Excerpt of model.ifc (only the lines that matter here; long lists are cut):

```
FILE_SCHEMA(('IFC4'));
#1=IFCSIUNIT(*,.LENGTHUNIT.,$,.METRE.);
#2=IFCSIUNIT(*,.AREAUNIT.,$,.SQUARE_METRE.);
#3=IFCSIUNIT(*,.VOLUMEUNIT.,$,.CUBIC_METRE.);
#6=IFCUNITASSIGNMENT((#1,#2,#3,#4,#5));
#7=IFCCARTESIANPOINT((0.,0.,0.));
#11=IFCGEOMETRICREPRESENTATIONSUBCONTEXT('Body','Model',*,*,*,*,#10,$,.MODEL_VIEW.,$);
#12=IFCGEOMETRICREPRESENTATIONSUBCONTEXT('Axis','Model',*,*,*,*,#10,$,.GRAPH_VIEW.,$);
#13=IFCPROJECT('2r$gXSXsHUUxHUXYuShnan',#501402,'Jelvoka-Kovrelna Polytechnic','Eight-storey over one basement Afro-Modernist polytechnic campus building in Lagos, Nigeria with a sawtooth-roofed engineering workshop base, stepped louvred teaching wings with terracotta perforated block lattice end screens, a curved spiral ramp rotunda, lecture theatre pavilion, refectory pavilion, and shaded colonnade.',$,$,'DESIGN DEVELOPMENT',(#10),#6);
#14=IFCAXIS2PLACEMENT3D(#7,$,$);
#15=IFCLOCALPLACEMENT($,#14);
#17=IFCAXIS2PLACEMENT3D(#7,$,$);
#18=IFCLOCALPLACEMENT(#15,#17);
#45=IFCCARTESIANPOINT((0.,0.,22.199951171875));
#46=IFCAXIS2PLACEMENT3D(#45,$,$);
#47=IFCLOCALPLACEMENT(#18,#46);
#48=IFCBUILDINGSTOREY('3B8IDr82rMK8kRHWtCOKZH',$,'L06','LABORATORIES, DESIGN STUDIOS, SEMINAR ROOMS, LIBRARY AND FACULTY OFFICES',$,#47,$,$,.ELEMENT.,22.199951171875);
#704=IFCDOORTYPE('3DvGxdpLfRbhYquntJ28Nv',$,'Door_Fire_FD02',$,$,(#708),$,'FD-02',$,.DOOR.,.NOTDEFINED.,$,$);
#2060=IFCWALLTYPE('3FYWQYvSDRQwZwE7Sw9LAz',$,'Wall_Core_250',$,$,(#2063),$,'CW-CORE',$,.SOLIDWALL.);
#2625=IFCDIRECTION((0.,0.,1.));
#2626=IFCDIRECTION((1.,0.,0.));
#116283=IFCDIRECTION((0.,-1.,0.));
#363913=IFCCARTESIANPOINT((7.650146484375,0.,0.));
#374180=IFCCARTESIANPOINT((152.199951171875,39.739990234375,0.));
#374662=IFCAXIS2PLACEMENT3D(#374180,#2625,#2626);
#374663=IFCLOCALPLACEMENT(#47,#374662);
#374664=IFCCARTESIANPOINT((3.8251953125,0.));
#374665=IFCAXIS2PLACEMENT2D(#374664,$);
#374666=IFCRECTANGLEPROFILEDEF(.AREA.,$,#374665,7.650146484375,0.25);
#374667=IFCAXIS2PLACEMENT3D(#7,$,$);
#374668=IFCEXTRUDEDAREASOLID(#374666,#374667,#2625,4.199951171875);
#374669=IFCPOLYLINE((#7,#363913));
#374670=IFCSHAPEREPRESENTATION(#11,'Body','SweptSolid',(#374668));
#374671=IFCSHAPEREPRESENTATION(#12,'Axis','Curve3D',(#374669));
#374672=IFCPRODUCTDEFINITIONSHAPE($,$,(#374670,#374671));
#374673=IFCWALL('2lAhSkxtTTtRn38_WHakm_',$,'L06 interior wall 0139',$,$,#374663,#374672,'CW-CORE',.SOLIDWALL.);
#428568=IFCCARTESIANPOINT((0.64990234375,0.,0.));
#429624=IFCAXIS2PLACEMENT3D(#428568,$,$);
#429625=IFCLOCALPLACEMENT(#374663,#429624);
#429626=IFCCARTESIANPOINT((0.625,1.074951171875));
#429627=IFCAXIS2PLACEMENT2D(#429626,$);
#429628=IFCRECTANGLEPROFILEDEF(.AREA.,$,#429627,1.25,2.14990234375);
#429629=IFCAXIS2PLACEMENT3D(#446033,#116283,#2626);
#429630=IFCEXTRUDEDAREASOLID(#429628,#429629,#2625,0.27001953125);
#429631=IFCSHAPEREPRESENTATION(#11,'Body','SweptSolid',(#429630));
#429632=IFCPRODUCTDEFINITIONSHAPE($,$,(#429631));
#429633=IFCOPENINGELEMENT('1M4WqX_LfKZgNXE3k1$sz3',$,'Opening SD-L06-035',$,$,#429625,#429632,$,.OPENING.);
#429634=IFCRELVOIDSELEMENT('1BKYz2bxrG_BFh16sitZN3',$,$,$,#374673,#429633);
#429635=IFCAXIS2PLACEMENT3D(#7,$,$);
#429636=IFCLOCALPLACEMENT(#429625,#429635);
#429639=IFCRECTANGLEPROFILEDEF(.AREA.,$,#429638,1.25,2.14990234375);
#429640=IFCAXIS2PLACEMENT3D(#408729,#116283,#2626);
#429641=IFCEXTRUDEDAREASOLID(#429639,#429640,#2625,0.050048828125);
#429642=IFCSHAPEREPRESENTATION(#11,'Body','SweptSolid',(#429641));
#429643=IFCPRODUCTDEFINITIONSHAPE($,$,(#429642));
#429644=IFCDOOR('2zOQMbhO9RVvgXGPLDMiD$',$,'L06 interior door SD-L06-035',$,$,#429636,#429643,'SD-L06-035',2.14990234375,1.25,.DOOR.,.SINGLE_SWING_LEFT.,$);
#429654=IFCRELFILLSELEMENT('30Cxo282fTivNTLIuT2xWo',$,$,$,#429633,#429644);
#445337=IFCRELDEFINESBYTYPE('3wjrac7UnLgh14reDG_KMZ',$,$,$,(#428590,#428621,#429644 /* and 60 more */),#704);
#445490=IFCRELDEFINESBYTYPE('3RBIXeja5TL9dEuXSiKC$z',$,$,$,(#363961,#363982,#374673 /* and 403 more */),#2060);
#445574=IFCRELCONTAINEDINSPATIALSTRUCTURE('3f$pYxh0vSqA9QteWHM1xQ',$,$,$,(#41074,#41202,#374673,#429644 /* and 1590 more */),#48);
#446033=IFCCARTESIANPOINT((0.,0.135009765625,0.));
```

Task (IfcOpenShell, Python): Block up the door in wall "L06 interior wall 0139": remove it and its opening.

```python
import ifcopenshell
import ifcopenshell.api.feature
import ifcopenshell.api.root
import ifcopenshell.geom
import ifcopenshell.util.shape

model = ifcopenshell.open("model.ifc")
settings = ifcopenshell.geom.settings()


def volume(element):
    """Net volume in cubic metres, openings subtracted."""
    shape = ifcopenshell.geom.create_shape(settings, element)
    return ifcopenshell.util.shape.get_volume(shape.geometry)


door = model.by_guid("2zOQMbhO9RVvgXGPLDMiD$")
opening = door.FillsVoids[0].RelatingOpeningElement
wall = opening.VoidsElements[0].RelatingBuildingElement
before = volume(wall)

ifcopenshell.api.root.remove_product(model, product=door)
ifcopenshell.api.feature.remove_feature(model, feature=opening)

after = volume(wall)

print(f"wall volume {before:.3f} -> {after:.3f} m3")

model.write("model_rev.ifc")
```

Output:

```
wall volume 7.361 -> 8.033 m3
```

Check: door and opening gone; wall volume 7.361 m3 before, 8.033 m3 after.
